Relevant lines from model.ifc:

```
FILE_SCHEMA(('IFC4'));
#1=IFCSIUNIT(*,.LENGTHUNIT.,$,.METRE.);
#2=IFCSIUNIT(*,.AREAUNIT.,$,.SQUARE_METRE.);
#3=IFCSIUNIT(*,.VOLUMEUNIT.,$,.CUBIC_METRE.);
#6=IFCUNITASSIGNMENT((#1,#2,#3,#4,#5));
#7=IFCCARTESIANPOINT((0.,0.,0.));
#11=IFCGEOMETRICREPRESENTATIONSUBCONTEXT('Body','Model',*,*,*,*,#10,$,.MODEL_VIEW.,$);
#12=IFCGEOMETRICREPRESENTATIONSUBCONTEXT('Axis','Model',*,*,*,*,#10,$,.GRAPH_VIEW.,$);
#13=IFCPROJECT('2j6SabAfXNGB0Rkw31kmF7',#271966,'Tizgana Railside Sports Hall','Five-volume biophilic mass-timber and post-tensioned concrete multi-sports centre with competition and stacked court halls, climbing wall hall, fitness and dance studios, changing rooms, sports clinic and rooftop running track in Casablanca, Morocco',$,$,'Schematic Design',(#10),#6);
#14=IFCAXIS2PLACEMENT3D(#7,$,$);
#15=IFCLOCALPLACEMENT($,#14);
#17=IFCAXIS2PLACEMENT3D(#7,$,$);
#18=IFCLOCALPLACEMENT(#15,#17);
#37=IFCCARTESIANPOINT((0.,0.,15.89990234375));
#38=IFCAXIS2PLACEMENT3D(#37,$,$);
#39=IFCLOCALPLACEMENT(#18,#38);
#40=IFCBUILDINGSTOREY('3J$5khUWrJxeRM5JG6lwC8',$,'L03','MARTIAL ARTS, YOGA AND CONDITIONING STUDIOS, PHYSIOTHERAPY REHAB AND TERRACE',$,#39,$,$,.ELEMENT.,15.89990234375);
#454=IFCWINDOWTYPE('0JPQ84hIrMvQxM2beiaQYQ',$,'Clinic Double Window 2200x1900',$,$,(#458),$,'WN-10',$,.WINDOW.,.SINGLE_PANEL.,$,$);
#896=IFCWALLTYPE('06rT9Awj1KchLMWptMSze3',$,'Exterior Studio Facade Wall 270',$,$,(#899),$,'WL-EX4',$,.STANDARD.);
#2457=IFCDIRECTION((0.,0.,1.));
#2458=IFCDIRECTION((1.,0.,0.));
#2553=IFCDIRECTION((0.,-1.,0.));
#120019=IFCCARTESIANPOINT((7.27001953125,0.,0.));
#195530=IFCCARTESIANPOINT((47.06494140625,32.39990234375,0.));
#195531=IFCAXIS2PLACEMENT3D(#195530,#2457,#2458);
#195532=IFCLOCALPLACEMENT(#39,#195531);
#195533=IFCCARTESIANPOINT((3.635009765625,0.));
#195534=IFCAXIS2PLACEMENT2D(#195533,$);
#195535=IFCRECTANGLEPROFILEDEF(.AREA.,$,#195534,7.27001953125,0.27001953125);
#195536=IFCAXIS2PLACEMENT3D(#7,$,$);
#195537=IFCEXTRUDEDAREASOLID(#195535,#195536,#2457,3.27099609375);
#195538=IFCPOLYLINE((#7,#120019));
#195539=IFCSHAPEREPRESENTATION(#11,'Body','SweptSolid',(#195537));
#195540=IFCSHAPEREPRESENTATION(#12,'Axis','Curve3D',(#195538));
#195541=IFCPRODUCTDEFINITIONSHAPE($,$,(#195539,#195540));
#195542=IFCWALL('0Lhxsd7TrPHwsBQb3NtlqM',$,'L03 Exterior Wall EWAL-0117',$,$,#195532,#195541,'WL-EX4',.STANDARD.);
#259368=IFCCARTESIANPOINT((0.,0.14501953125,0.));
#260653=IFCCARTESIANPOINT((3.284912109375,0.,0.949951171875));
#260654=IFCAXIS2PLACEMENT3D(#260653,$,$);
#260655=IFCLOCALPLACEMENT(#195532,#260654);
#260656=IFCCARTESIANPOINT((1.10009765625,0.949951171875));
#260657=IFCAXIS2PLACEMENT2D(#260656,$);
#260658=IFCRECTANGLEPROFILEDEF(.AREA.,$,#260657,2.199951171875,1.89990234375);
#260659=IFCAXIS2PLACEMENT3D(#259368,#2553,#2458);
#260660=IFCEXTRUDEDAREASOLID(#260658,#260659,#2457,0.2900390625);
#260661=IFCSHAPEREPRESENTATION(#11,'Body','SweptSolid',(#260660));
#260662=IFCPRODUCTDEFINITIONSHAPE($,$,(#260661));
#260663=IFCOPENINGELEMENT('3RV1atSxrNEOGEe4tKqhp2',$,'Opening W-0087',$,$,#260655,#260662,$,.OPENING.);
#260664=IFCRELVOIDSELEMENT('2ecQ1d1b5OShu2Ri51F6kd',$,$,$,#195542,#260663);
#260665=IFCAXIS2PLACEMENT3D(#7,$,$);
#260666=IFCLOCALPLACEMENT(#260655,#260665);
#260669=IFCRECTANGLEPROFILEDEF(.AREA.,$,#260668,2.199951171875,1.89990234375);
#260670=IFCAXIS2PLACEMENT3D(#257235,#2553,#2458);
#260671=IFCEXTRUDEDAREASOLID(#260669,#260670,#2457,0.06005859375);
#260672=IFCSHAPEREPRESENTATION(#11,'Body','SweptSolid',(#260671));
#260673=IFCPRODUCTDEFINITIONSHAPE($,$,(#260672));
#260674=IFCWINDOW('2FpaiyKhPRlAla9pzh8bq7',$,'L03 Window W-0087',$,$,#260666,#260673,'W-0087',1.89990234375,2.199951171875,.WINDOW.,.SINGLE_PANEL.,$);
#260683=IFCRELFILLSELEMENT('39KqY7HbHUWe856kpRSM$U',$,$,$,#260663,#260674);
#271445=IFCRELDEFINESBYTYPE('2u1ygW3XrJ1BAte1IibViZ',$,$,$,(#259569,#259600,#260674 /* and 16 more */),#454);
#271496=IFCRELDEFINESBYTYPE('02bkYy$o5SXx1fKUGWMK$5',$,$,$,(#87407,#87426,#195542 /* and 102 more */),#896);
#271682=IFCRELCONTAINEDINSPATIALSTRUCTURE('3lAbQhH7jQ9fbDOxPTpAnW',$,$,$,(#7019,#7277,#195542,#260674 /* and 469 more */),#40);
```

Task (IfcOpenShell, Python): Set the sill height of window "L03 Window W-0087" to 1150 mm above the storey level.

```python
import numpy as np
import ifcopenshell
import ifcopenshell.api.geometry
import ifcopenshell.geom
import ifcopenshell.util.element
import ifcopenshell.util.placement
import ifcopenshell.util.shape
import ifcopenshell.util.unit

model = ifcopenshell.open("model.ifc")
unit_scale = ifcopenshell.util.unit.calculate_unit_scale(model)

window = model.by_guid("2FpaiyKhPRlAla9pzh8bq7")
opening = window.FillsVoids[0].RelatingOpeningElement
storey = ifcopenshell.util.element.get_container(window, ifc_class="IfcBuildingStorey")
level = ifcopenshell.util.placement.get_local_placement(storey.ObjectPlacement)[2, 3]

# The opening's origin need not be at the sill, so measure its lowest point.
shape = ifcopenshell.geom.create_shape(ifcopenshell.geom.settings(), opening)
bottom = ifcopenshell.util.shape.get_shape_bottom_elevation(shape, shape.geometry) / unit_scale
dz = level + 1.15 / unit_scale - bottom

shift = np.array([0.0, 0.0, dz])
# The window is placed relative to its opening, so it follows when the opening moves.
matrix = ifcopenshell.util.placement.get_local_placement(opening.ObjectPlacement)
matrix[:3, 3] += shift
ifcopenshell.api.geometry.edit_object_placement(
    model, product=opening, matrix=matrix, is_si=False, should_transform_children=True
)

print(f"moved by {dz * unit_scale:+.3f} m")

model.write("model-out.ifc")
```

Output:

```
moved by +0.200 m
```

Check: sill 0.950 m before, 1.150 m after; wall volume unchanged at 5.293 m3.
